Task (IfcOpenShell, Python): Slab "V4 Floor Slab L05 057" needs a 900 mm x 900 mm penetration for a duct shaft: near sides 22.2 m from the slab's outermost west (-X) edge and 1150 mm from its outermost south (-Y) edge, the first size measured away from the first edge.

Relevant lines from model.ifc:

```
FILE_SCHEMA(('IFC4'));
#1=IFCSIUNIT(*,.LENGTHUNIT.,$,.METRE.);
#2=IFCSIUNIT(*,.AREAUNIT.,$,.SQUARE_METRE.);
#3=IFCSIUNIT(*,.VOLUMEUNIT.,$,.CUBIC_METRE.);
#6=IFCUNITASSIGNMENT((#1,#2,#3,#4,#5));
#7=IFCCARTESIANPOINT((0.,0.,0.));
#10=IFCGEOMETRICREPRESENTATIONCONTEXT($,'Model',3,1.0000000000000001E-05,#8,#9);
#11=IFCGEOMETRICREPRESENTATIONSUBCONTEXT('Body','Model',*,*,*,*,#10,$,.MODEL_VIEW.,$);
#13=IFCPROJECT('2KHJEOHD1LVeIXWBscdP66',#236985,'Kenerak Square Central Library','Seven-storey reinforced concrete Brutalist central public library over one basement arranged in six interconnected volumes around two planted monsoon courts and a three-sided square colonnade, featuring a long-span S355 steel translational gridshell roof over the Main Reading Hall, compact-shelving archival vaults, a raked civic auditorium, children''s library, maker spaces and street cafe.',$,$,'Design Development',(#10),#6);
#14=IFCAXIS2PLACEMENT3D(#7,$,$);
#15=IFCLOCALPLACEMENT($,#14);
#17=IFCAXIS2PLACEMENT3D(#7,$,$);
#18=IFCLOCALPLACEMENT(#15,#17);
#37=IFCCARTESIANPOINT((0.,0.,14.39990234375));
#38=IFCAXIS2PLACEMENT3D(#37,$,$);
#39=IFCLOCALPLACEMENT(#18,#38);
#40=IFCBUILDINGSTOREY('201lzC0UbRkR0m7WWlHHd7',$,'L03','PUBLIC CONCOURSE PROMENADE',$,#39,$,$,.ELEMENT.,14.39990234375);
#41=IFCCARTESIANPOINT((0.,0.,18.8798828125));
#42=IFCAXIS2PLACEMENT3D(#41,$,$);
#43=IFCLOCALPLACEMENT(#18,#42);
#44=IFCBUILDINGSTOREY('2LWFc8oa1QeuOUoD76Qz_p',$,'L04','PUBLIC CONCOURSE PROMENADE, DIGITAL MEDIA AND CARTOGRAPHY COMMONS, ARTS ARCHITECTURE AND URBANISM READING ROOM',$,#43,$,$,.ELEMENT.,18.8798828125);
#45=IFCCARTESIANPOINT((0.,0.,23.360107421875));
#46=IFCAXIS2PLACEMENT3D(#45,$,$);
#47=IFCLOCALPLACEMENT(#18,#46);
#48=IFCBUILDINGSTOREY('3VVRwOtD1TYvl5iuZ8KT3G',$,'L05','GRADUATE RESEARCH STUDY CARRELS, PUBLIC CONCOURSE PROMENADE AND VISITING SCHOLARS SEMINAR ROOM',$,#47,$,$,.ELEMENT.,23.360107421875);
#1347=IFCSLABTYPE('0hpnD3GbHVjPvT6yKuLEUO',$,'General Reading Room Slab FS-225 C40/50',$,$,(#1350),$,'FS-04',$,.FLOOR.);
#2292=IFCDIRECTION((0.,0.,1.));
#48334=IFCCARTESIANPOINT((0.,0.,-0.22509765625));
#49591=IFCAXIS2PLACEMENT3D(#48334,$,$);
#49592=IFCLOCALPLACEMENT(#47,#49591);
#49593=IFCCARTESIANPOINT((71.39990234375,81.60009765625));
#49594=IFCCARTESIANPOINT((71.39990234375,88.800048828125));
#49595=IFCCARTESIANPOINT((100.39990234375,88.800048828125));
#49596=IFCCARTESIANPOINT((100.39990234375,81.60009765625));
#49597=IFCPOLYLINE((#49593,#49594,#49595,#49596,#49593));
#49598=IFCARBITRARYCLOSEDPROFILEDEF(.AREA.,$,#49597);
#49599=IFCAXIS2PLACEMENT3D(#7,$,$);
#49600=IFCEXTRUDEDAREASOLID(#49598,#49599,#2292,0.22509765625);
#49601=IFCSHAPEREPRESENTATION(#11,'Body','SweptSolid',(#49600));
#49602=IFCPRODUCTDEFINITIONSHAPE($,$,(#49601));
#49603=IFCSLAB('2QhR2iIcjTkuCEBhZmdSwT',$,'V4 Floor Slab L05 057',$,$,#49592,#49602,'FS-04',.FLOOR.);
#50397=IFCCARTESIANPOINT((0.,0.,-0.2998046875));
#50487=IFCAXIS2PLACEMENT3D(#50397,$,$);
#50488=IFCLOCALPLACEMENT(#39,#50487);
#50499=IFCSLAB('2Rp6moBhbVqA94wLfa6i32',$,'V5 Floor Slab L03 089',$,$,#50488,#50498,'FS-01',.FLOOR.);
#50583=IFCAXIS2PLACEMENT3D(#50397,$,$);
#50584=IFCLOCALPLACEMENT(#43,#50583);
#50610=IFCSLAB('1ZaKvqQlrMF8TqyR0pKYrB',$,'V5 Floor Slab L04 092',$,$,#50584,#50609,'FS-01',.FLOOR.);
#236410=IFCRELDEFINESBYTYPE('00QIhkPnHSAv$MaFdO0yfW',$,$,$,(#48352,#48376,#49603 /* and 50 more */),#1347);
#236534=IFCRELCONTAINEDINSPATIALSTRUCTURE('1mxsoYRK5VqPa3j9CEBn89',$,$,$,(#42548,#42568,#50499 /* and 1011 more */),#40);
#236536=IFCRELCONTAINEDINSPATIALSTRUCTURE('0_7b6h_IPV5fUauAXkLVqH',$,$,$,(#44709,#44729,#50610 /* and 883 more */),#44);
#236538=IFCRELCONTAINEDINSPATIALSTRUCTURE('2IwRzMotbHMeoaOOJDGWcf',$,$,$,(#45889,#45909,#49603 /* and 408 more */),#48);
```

```python
import numpy as np
import ifcopenshell
import ifcopenshell.api.feature
import ifcopenshell.api.geometry
import ifcopenshell.api.root
import ifcopenshell.geom
import ifcopenshell.util.placement
import ifcopenshell.util.representation
import ifcopenshell.util.shape
import ifcopenshell.util.unit

model = ifcopenshell.open("model.ifc")
unit_scale = ifcopenshell.util.unit.calculate_unit_scale(model)
settings = ifcopenshell.geom.settings()


def volume(element):
    """Net volume in cubic metres, openings subtracted."""
    shape = ifcopenshell.geom.create_shape(settings, element)
    return ifcopenshell.util.shape.get_volume(shape.geometry)


slab = model.by_guid("2QhR2iIcjTkuCEBhZmdSwT")
before = volume(slab)

# Extent in the slab's own axes, in metres. The edges named are its -X and -Y sides.
slab_shape = ifcopenshell.geom.create_shape(settings, slab)
vertices = ifcopenshell.util.shape.get_vertices(slab_shape.geometry)
x_min, y_min, bottom = vertices.min(axis=0)
top = vertices[:, 2].max()

opening = ifcopenshell.api.root.create_entity(model, ifc_class="IfcOpeningElement", name="Duct shaft opening", predefined_type="OPENING")
context = ifcopenshell.util.representation.get_context(model, "Model", "Body", "MODEL_VIEW")
width, depth = 0.9, 0.9
outline = [(0.0, 0.0), (width, 0.0), (width, depth), (0.0, depth), (0.0, 0.0)]
# Overshoot both faces by 50 mm so the cut is clean.
shape = ifcopenshell.api.geometry.add_slab_representation(
    model, context=context, depth=top - bottom + 0.1, polyline=outline
)
ifcopenshell.api.geometry.assign_representation(model, product=opening, representation=shape)

matrix = ifcopenshell.util.placement.get_local_placement(slab.ObjectPlacement)
matrix[:, 3] = matrix @ np.append(np.array([x_min + 22.2, y_min + 1.15, bottom - 0.05]) / unit_scale, 1.0)
ifcopenshell.api.geometry.edit_object_placement(model, product=opening, matrix=matrix, is_si=False)
ifcopenshell.api.feature.add_feature(model, feature=opening, element=slab)

after = volume(slab)

print(f"slab volume {before:.3f} -> {after:.3f} m3")

model.write("model_v2.ifc")
```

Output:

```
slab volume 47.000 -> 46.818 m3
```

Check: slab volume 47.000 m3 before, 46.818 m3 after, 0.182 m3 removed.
